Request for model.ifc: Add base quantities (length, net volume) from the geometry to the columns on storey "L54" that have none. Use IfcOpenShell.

First a look at what the model holds.

```python
import ifcopenshell
import ifcopenshell.util.element
import ifcopenshell.util.unit

model = ifcopenshell.open("model.ifc")
print(model.schema)
for unit_type in ("LENGTHUNIT", "AREAUNIT", "VOLUMEUNIT"):
    print(unit_type, ifcopenshell.util.unit.calculate_unit_scale(model, unit_type))
storey = next(s for s in model.by_type("IfcBuildingStorey") if s.Name == "L54")
columns = [e for e in ifcopenshell.util.element.get_decomposition(storey) if e.is_a("IfcColumn")]
for e in sorted(columns, key=lambda e: e.id()):
    print(e.id(), e.is_a(), e.Name, list(ifcopenshell.util.element.get_psets(e, qtos_only=True)), sep=" | ")
```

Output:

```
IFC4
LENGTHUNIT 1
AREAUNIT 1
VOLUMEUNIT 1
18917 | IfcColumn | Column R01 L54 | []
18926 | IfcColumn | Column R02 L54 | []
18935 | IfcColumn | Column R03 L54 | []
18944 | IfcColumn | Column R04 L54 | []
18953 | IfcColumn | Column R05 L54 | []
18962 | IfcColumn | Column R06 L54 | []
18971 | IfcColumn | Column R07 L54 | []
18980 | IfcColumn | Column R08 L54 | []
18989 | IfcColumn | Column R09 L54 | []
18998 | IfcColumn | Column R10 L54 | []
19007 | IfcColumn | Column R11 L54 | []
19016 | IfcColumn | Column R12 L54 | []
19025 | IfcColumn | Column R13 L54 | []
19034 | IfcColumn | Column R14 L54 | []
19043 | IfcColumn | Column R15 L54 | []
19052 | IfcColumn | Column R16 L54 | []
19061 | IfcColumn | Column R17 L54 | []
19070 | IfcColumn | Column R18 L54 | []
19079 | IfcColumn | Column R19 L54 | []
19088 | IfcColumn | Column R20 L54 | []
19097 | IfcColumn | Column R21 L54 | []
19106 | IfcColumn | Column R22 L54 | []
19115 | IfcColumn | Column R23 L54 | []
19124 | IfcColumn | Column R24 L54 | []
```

```python
import ifcopenshell
import ifcopenshell.api.pset
import ifcopenshell.geom
import ifcopenshell.util.element
import ifcopenshell.util.shape
import ifcopenshell.util.unit

model = ifcopenshell.open("model.ifc")
unit_scale = ifcopenshell.util.unit.calculate_unit_scale(model)
volume_scale = ifcopenshell.util.unit.calculate_unit_scale(model, "VOLUMEUNIT")
settings = ifcopenshell.geom.settings()

storey = next(s for s in model.by_type("IfcBuildingStorey") if s.Name == "L54")
columns = [e for e in ifcopenshell.util.element.get_decomposition(storey) if e.is_a("IfcColumn")]

for e in sorted(columns, key=lambda e: e.id()):
    if ifcopenshell.util.element.get_psets(e, qtos_only=True, should_inherit=False):
        continue
    # Geometry comes back in metres, in the element's own axes.
    shape = ifcopenshell.geom.create_shape(settings, e)
    values = {
        "Length": ifcopenshell.util.shape.get_z(shape.geometry) / unit_scale,
        "NetVolume": ifcopenshell.util.shape.get_volume(shape.geometry) / volume_scale,
    }
    qto = ifcopenshell.api.pset.add_qto(model, product=e, name="Qto_ColumnBaseQuantities")
    ifcopenshell.api.pset.edit_qto(model, qto=qto, properties=values)
    print(e.id(), {k: round(v, 3) for k, v in values.items()})

model.write("model_edited.ifc")
```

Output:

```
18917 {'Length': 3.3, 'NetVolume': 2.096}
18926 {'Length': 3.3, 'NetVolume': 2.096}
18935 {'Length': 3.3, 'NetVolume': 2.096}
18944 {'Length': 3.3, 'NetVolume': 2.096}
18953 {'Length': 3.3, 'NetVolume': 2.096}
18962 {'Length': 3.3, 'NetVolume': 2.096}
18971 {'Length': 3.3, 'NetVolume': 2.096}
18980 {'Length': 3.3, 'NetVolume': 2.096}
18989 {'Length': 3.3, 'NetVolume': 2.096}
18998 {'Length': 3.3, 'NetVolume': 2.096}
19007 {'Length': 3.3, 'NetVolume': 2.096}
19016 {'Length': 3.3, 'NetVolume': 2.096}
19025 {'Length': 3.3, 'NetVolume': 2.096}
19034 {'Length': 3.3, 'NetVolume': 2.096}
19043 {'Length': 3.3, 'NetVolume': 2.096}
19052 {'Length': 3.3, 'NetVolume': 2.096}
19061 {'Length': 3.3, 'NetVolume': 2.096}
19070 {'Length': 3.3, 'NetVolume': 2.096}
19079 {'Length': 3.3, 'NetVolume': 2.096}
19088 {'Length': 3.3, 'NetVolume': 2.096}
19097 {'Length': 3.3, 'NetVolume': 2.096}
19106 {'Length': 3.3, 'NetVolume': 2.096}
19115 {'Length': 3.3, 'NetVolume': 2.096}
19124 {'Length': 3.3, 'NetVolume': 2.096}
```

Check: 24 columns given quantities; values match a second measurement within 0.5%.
